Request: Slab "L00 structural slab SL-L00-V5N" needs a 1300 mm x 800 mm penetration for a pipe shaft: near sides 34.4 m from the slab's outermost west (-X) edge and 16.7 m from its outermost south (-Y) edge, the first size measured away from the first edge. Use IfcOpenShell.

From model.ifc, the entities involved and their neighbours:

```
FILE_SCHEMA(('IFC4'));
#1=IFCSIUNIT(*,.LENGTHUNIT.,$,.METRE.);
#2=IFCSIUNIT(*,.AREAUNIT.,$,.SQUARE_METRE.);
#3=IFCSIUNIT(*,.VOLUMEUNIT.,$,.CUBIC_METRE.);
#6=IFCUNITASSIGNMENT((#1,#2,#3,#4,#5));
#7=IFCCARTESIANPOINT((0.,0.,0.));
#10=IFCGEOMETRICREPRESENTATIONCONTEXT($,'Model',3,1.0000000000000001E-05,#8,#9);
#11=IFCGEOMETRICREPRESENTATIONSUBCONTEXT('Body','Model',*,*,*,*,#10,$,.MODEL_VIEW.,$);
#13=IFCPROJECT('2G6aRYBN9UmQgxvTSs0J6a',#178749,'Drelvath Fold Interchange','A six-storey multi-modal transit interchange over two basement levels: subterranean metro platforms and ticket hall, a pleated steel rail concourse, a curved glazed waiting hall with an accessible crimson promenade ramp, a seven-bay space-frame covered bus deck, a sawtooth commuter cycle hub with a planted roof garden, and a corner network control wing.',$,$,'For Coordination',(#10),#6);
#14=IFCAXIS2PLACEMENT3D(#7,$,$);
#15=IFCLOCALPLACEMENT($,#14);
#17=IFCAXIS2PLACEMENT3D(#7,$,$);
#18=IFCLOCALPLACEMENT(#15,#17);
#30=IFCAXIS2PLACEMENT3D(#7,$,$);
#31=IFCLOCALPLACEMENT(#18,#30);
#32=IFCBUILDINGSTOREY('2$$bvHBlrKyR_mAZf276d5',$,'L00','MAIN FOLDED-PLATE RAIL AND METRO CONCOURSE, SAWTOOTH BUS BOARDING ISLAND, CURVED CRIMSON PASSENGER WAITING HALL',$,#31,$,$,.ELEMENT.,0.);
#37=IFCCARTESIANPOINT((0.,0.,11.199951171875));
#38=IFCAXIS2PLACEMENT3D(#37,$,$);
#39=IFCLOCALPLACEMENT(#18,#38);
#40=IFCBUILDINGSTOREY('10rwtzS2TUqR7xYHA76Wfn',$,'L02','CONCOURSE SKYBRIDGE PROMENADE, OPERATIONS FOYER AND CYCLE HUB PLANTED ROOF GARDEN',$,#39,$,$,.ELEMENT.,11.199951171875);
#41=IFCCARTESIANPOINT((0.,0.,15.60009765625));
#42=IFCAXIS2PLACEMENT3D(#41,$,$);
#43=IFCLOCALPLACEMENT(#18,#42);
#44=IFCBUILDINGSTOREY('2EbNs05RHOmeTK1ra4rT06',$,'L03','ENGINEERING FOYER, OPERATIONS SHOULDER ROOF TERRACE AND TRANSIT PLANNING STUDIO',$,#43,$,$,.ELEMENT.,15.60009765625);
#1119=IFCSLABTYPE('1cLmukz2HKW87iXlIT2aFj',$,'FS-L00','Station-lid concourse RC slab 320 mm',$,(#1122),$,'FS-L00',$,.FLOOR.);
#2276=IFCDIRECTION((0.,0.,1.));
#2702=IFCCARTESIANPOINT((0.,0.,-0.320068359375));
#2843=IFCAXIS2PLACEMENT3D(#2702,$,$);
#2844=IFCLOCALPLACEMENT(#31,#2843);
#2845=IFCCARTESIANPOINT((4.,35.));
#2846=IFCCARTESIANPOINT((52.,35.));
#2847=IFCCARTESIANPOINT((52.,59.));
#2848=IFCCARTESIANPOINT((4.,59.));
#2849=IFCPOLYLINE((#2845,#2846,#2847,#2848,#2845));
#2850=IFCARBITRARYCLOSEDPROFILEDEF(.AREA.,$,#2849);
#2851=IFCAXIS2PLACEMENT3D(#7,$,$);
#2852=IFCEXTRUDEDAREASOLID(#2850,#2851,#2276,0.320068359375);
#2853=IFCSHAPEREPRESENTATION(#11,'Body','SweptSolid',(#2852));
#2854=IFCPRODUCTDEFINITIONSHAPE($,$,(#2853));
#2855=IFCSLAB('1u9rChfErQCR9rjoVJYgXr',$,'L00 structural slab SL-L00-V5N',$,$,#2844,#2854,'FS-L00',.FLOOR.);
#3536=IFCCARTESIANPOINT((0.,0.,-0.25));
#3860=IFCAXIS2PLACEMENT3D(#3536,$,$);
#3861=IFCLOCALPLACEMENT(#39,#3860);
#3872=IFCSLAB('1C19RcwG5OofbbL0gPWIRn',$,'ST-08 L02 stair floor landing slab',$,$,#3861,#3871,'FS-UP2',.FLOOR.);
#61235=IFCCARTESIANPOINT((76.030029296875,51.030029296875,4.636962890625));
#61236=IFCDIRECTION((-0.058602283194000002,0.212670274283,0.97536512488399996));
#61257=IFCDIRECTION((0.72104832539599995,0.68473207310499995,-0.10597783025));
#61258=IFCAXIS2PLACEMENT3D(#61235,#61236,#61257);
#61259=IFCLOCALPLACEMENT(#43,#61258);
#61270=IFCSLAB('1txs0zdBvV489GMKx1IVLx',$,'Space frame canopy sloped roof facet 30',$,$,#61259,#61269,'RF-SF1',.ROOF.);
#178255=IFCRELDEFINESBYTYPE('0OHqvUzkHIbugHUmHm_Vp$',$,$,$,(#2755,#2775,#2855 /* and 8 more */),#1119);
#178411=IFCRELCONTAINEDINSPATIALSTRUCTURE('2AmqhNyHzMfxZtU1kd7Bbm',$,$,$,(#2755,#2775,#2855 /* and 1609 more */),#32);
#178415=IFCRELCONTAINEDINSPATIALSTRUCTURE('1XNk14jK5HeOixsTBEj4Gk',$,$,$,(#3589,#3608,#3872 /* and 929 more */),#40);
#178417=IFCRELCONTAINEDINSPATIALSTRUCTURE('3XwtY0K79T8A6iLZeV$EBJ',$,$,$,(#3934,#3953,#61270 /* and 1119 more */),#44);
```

```python
import numpy as np
import ifcopenshell
import ifcopenshell.api.feature
import ifcopenshell.api.geometry
import ifcopenshell.api.root
import ifcopenshell.geom
import ifcopenshell.util.placement
import ifcopenshell.util.representation
import ifcopenshell.util.shape
import ifcopenshell.util.unit

model = ifcopenshell.open("model.ifc")
unit_scale = ifcopenshell.util.unit.calculate_unit_scale(model)
settings = ifcopenshell.geom.settings()


def volume(element):
    """Net volume in cubic metres, openings subtracted."""
    shape = ifcopenshell.geom.create_shape(settings, element)
    return ifcopenshell.util.shape.get_volume(shape.geometry)


slab = model.by_id(2855)
before = volume(slab)

# Extent in the slab's own axes, in metres. The edges named are its -X and -Y sides.
slab_shape = ifcopenshell.geom.create_shape(settings, slab)
vertices = ifcopenshell.util.shape.get_vertices(slab_shape.geometry)
x_min, y_min, bottom = vertices.min(axis=0)
top = vertices[:, 2].max()

opening = ifcopenshell.api.root.create_entity(model, ifc_class="IfcOpeningElement", name="Pipe shaft opening", predefined_type="OPENING")
context = ifcopenshell.util.representation.get_context(model, "Model", "Body", "MODEL_VIEW")
width, depth = 1.3, 0.8
outline = [(0.0, 0.0), (width, 0.0), (width, depth), (0.0, depth), (0.0, 0.0)]
# Overshoot both faces by 50 mm so the cut is clean.
shape = ifcopenshell.api.geometry.add_slab_representation(
    model, context=context, depth=top - bottom + 0.1, polyline=outline
)
ifcopenshell.api.geometry.assign_representation(model, product=opening, representation=shape)

matrix = ifcopenshell.util.placement.get_local_placement(slab.ObjectPlacement)
matrix[:, 3] = matrix @ np.append(np.array([x_min + 34.4, y_min + 16.7, bottom - 0.05]) / unit_scale, 1.0)
ifcopenshell.api.geometry.edit_object_placement(model, product=opening, matrix=matrix, is_si=False)
ifcopenshell.api.feature.add_feature(model, feature=opening, element=slab)

after = volume(slab)

print(f"slab volume {before:.3f} -> {after:.3f} m3")

model.write("model_updated.ifc")
```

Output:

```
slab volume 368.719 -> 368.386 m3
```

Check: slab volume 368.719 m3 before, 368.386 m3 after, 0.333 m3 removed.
